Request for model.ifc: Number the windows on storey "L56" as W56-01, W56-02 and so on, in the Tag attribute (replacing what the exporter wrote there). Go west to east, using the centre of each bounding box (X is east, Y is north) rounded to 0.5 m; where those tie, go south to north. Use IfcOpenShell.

First a look at what the model holds.

```python
import ifcopenshell
import ifcopenshell.util.element
import ifcopenshell.util.placement

model = ifcopenshell.open("model.ifc")
print(model.schema)
storey = next(s for s in model.by_type("IfcBuildingStorey") if s.Name == "L56")
windows = [e for e in ifcopenshell.util.element.get_decomposition(storey) if e.is_a("IfcWindow")]
for e in sorted(windows, key=lambda e: e.id()):
    origin = ifcopenshell.util.placement.get_local_placement(e.ObjectPlacement)[:3, 3]
    print(e.id(), e.Tag, e.Name, origin.round(2) + 0.0, sep=" | ")
```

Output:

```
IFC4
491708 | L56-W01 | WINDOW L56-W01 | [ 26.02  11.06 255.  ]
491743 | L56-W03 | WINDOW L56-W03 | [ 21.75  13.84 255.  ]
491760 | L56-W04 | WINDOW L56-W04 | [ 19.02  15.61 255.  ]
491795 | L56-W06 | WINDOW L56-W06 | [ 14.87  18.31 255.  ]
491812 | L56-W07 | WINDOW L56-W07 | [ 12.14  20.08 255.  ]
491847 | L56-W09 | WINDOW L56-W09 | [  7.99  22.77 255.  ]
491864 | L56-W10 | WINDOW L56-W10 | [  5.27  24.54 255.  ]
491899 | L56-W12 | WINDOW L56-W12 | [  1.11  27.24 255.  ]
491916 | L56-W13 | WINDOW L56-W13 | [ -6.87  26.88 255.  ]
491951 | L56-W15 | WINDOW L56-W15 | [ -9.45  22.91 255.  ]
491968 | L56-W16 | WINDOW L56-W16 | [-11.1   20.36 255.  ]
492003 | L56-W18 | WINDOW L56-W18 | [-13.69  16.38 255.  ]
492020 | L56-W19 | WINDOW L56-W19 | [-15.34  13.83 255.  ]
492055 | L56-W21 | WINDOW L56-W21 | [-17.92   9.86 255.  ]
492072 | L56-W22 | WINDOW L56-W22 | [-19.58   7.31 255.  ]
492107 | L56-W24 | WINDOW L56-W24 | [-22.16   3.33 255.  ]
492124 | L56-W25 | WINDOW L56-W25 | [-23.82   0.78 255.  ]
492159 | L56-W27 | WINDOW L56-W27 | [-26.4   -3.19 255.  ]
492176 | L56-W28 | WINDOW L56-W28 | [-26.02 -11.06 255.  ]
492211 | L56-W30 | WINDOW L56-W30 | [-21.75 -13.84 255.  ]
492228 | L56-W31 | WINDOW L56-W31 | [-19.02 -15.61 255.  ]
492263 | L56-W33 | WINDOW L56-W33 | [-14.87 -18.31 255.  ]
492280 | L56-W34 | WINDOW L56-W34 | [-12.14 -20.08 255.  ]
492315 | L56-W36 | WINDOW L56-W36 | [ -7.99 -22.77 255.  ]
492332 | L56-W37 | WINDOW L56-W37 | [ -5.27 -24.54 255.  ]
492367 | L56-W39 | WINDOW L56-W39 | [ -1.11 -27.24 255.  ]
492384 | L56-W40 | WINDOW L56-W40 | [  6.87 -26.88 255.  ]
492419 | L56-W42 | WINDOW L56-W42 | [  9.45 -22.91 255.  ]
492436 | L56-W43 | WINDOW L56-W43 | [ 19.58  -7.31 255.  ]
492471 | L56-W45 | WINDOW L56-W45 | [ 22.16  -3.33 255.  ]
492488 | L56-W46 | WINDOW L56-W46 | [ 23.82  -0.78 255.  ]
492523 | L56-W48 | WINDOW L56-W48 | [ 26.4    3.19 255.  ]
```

```python
import ifcopenshell
import ifcopenshell.geom
import ifcopenshell.util.element
import ifcopenshell.util.shape

model = ifcopenshell.open("model.ifc")
settings = ifcopenshell.geom.settings()
settings.set("use-world-coords", True)


def centre(element):
    shape = ifcopenshell.geom.create_shape(settings, element)
    return ifcopenshell.util.shape.get_bbox_centroid(shape.geometry)


storey = next(s for s in model.by_type("IfcBuildingStorey") if s.Name == "L56")
windows = [e for e in ifcopenshell.util.element.get_decomposition(storey) if e.is_a("IfcWindow")]

# Insertion points can sit at a corner or the storey origin, so sort by the geometry (in metres).
centres = {e: centre(e) for e in windows}
windows.sort(key=lambda e: (round(centres[e][0] / 0.5), centres[e][1]))

for i, e in enumerate(windows, start=1):
    number = f"W56-{i:02d}"
    e.Tag = number
    print(e.id(), number)

model.write("model_v2.ifc")
```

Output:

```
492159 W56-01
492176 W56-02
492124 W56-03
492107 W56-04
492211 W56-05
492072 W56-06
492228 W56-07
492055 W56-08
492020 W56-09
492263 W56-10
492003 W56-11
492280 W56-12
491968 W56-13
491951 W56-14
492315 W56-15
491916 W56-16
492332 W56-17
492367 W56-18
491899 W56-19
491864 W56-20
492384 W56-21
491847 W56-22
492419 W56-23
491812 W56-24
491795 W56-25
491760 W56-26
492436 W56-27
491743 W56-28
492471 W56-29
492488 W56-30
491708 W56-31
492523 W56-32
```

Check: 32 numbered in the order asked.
